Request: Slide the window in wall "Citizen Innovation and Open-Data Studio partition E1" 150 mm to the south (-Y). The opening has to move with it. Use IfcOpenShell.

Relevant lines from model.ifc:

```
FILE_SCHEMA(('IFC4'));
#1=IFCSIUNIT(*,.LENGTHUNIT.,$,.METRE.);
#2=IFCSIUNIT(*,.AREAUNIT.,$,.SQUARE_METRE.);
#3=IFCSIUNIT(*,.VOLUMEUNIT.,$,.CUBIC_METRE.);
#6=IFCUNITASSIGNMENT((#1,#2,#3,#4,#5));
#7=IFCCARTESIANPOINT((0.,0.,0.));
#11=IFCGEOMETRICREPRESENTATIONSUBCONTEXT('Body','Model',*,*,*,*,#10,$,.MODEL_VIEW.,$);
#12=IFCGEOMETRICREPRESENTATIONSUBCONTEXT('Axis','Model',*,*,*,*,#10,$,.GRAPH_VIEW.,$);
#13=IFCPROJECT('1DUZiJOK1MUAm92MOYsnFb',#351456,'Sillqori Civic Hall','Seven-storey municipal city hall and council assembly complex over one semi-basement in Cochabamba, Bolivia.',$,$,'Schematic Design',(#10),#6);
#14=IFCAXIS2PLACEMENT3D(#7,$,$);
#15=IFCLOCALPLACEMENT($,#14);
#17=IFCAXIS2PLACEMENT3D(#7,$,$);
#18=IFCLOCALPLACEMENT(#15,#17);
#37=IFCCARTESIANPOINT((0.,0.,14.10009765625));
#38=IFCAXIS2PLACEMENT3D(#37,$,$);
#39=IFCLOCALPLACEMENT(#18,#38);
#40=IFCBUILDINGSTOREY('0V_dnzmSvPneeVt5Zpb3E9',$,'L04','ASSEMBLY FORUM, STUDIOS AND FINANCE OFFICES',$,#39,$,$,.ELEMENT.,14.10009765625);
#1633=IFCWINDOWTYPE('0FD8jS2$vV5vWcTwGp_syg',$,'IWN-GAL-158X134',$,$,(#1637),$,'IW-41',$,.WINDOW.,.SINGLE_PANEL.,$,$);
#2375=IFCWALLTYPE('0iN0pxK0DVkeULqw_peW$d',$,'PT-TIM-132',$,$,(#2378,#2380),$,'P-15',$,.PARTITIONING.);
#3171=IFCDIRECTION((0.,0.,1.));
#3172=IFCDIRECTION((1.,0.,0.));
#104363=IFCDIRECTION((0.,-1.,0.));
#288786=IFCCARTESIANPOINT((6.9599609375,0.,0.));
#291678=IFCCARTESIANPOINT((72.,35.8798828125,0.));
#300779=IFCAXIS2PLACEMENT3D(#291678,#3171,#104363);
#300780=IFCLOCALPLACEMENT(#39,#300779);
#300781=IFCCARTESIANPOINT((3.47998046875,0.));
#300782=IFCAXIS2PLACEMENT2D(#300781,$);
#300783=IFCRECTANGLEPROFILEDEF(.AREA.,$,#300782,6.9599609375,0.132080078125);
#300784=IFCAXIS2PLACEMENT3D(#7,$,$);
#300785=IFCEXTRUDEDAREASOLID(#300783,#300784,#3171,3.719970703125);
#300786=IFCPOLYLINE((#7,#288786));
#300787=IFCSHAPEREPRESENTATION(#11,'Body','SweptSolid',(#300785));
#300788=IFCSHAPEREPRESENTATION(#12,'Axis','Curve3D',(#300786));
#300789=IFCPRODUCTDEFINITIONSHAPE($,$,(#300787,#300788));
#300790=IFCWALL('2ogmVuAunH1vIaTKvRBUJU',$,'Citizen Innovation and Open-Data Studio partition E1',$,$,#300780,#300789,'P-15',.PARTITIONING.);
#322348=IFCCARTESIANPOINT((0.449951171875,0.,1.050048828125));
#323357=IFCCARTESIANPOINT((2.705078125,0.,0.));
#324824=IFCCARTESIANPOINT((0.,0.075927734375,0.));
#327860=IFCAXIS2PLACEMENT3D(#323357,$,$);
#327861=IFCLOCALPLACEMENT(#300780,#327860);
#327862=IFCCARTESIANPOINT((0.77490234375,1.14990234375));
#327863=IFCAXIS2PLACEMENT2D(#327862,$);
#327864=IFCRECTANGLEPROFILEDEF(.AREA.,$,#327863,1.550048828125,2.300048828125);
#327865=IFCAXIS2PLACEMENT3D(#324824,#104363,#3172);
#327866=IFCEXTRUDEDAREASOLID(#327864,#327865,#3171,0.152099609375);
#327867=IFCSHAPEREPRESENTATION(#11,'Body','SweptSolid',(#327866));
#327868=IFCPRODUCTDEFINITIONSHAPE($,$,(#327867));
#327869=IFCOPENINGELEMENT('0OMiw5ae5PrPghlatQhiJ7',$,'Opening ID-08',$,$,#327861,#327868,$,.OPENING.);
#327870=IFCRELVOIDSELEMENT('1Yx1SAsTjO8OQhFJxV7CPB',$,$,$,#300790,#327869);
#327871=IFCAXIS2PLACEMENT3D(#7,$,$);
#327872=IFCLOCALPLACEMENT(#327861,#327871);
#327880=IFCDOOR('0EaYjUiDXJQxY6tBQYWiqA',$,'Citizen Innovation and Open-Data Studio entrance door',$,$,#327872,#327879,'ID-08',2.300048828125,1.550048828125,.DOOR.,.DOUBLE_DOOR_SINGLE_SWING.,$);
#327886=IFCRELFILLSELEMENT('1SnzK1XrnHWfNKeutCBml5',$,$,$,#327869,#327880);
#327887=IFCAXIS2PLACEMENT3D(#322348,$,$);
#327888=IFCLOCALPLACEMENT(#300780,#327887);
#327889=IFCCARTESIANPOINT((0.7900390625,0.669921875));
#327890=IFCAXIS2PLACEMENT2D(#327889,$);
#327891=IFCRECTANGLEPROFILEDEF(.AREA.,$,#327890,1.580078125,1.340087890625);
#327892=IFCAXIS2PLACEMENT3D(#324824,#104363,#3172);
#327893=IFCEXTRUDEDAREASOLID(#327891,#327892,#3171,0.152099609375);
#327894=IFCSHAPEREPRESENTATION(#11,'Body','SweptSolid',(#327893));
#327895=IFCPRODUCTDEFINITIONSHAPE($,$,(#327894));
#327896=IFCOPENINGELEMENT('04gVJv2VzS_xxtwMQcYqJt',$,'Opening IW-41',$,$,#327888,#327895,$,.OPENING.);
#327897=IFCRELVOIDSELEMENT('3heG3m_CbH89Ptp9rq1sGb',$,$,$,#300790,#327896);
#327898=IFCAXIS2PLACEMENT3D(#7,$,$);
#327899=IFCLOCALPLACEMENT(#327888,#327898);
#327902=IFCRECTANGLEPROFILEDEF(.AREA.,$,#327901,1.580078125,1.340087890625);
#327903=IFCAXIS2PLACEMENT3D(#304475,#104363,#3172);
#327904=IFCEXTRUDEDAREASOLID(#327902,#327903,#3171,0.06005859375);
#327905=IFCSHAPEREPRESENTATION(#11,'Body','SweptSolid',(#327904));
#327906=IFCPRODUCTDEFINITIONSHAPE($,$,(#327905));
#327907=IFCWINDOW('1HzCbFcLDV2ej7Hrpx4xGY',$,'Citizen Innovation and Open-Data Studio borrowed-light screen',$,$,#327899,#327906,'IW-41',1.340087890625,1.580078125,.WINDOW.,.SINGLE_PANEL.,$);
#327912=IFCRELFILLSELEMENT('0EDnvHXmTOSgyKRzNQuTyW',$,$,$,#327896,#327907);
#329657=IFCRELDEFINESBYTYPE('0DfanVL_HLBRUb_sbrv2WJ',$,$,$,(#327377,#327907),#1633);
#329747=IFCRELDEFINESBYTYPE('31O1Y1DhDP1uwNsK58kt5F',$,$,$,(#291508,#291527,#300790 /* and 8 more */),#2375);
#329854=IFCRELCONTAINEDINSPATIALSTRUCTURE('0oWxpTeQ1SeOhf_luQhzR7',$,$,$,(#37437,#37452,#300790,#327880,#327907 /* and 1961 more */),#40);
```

```python
import ifcopenshell
import ifcopenshell.api.geometry
import ifcopenshell.util.placement
import ifcopenshell.util.unit

model = ifcopenshell.open("model.ifc")
unit_scale = ifcopenshell.util.unit.calculate_unit_scale(model)

window = model.by_guid("1HzCbFcLDV2ej7Hrpx4xGY")
opening = window.FillsVoids[0].RelatingOpeningElement
wall = opening.VoidsElements[0].RelatingBuildingElement

wall_matrix = ifcopenshell.util.placement.get_local_placement(wall.ObjectPlacement)
shift = wall_matrix[:3, 0] * 0.15 / unit_scale
before = ifcopenshell.util.placement.get_local_placement(window.ObjectPlacement)[:3, 3].copy()

# The window is placed relative to its opening, so it follows when the opening moves.
matrix = ifcopenshell.util.placement.get_local_placement(opening.ObjectPlacement)
matrix[:3, 3] += shift
ifcopenshell.api.geometry.edit_object_placement(
    model, product=opening, matrix=matrix, is_si=False, should_transform_children=True
)

after = ifcopenshell.util.placement.get_local_placement(window.ObjectPlacement)[:3, 3]
print("window moved by", (after - before).round(3) + 0.0)

model.write("model_updated.ifc")
```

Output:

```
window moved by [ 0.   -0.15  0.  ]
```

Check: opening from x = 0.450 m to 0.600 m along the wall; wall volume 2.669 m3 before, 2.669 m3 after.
